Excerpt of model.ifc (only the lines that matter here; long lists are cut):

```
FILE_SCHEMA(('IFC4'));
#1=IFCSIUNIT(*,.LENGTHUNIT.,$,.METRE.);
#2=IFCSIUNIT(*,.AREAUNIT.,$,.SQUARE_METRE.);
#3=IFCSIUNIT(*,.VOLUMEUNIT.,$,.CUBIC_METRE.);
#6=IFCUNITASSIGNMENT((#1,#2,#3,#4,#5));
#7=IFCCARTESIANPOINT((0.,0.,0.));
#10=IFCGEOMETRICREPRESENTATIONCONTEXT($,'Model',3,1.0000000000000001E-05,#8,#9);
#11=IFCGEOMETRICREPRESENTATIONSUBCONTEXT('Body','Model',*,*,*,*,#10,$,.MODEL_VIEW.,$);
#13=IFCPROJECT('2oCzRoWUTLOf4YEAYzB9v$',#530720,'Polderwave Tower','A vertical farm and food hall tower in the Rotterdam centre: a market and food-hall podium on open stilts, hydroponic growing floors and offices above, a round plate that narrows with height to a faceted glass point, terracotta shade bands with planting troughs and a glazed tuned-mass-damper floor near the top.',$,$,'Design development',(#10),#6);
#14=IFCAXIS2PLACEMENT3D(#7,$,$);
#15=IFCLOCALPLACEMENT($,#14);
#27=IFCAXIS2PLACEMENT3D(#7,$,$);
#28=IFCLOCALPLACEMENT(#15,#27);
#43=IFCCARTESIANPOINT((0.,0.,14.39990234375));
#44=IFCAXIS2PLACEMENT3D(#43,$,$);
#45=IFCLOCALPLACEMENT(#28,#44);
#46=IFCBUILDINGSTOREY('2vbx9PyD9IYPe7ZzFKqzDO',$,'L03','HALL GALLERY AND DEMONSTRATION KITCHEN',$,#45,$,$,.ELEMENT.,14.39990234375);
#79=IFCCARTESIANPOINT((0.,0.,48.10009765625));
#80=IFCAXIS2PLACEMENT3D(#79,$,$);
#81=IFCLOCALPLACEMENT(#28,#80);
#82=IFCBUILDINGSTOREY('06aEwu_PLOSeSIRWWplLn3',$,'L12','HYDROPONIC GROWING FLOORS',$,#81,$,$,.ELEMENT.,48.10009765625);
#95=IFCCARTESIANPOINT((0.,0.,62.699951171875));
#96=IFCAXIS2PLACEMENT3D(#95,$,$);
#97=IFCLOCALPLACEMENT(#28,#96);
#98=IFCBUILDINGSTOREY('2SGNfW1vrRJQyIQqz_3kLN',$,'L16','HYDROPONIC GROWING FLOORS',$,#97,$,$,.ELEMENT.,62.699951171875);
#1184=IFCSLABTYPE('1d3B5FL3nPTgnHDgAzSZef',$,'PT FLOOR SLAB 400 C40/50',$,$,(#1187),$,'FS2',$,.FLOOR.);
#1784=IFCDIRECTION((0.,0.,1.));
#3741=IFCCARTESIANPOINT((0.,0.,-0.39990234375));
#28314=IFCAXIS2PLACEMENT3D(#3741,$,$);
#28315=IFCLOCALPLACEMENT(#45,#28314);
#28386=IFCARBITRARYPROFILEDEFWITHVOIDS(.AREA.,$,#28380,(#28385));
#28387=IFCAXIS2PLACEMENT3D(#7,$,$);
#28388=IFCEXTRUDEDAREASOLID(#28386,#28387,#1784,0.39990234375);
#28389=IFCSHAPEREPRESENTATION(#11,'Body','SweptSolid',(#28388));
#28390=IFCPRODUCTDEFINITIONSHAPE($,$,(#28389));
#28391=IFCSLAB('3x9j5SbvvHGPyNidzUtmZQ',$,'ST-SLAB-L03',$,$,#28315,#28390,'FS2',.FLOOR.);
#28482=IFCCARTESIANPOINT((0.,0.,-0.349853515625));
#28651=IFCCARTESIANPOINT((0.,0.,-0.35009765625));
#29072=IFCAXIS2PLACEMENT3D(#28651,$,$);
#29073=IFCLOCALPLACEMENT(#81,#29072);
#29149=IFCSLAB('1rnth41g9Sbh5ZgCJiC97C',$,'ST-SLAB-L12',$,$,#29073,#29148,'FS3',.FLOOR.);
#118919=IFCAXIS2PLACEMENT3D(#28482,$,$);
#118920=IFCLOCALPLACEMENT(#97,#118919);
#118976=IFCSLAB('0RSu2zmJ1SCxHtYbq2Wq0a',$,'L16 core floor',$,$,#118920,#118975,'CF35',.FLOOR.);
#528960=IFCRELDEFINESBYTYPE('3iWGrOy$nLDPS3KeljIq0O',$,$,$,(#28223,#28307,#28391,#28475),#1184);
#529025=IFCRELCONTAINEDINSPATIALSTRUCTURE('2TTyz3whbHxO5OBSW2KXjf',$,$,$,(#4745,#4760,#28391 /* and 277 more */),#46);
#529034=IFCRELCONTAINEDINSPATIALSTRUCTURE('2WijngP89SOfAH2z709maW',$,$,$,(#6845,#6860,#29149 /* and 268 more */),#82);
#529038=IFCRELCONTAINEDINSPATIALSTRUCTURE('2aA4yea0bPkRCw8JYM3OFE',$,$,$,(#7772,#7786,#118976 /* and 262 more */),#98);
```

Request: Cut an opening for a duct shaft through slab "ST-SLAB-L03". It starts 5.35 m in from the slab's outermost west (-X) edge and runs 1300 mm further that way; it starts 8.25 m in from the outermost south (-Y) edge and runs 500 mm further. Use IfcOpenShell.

```python
import numpy as np
import ifcopenshell
import ifcopenshell.api.feature
import ifcopenshell.api.geometry
import ifcopenshell.api.root
import ifcopenshell.geom
import ifcopenshell.util.placement
import ifcopenshell.util.representation
import ifcopenshell.util.shape
import ifcopenshell.util.unit

model = ifcopenshell.open("model.ifc")
unit_scale = ifcopenshell.util.unit.calculate_unit_scale(model)
settings = ifcopenshell.geom.settings()


def volume(element):
    """Net volume in cubic metres, openings subtracted."""
    shape = ifcopenshell.geom.create_shape(settings, element)
    return ifcopenshell.util.shape.get_volume(shape.geometry)


slab = model.by_id(28391)
before = volume(slab)

# Extent in the slab's own axes, in metres. The edges named are its -X and -Y sides.
slab_shape = ifcopenshell.geom.create_shape(settings, slab)
vertices = ifcopenshell.util.shape.get_vertices(slab_shape.geometry)
x_min, y_min, bottom = vertices.min(axis=0)
top = vertices[:, 2].max()

opening = ifcopenshell.api.root.create_entity(model, ifc_class="IfcOpeningElement", name="Duct shaft opening", predefined_type="OPENING")
context = ifcopenshell.util.representation.get_context(model, "Model", "Body", "MODEL_VIEW")
width, depth = 1.3, 0.5
outline = [(0.0, 0.0), (width, 0.0), (width, depth), (0.0, depth), (0.0, 0.0)]
# Overshoot both faces by 50 mm so the cut is clean.
shape = ifcopenshell.api.geometry.add_slab_representation(
    model, context=context, depth=top - bottom + 0.1, polyline=outline
)
ifcopenshell.api.geometry.assign_representation(model, product=opening, representation=shape)

matrix = ifcopenshell.util.placement.get_local_placement(slab.ObjectPlacement)
matrix[:, 3] = matrix @ np.append(np.array([x_min + 5.35, y_min + 8.25, bottom - 0.05]) / unit_scale, 1.0)
ifcopenshell.api.geometry.edit_object_placement(model, product=opening, matrix=matrix, is_si=False)
ifcopenshell.api.feature.add_feature(model, feature=opening, element=slab)

after = volume(slab)

print(f"slab volume {before:.3f} -> {after:.3f} m3")

model.write("model_updated.ifc")
```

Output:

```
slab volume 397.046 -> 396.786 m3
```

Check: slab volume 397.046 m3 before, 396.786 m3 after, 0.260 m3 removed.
